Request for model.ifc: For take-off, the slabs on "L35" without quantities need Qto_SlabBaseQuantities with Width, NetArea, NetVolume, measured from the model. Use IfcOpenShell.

First a look at what the model holds.

```python
import ifcopenshell
import ifcopenshell.util.element
import ifcopenshell.util.unit

model = ifcopenshell.open("model.ifc")
print(model.schema)
for unit_type in ("LENGTHUNIT", "AREAUNIT", "VOLUMEUNIT"):
    print(unit_type, ifcopenshell.util.unit.calculate_unit_scale(model, unit_type))
storey = next(s for s in model.by_type("IfcBuildingStorey") if s.Name == "L35")
slabs = [e for e in ifcopenshell.util.element.get_decomposition(storey) if e.is_a("IfcSlab")]
for e in sorted(slabs, key=lambda e: e.id()):
    print(e.id(), e.is_a(), e.Name, list(ifcopenshell.util.element.get_psets(e, qtos_only=True)), sep=" | ")
```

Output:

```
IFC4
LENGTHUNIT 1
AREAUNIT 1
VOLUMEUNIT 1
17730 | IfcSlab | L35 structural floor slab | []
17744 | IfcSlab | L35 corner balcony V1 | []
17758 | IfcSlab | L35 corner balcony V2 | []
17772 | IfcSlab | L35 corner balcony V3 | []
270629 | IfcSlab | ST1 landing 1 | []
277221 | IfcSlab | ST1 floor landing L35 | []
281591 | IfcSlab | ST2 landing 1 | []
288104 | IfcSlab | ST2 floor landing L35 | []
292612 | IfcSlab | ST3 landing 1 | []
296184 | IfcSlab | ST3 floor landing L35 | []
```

```python
import ifcopenshell
import ifcopenshell.api.pset
import ifcopenshell.geom
import ifcopenshell.util.element
import ifcopenshell.util.shape
import ifcopenshell.util.unit

model = ifcopenshell.open("model.ifc")
unit_scale = ifcopenshell.util.unit.calculate_unit_scale(model)
area_scale = ifcopenshell.util.unit.calculate_unit_scale(model, "AREAUNIT")
volume_scale = ifcopenshell.util.unit.calculate_unit_scale(model, "VOLUMEUNIT")
settings = ifcopenshell.geom.settings()

storey = next(s for s in model.by_type("IfcBuildingStorey") if s.Name == "L35")
slabs = [e for e in ifcopenshell.util.element.get_decomposition(storey) if e.is_a("IfcSlab")]

for e in sorted(slabs, key=lambda e: e.id()):
    if ifcopenshell.util.element.get_psets(e, qtos_only=True, should_inherit=False):
        continue
    # Geometry comes back in metres, in the element's own axes.
    shape = ifcopenshell.geom.create_shape(settings, e)
    values = {
        "Width": ifcopenshell.util.shape.get_z(shape.geometry) / unit_scale,
        "NetArea": ifcopenshell.util.shape.get_footprint_area(shape.geometry) / area_scale,
        "NetVolume": ifcopenshell.util.shape.get_volume(shape.geometry) / volume_scale,
    }
    qto = ifcopenshell.api.pset.add_qto(model, product=e, name="Qto_SlabBaseQuantities")
    ifcopenshell.api.pset.edit_qto(model, qto=qto, properties=values)
    print(e.id(), {k: round(v, 3) for k, v in values.items()})

model.write("model-out.ifc")
```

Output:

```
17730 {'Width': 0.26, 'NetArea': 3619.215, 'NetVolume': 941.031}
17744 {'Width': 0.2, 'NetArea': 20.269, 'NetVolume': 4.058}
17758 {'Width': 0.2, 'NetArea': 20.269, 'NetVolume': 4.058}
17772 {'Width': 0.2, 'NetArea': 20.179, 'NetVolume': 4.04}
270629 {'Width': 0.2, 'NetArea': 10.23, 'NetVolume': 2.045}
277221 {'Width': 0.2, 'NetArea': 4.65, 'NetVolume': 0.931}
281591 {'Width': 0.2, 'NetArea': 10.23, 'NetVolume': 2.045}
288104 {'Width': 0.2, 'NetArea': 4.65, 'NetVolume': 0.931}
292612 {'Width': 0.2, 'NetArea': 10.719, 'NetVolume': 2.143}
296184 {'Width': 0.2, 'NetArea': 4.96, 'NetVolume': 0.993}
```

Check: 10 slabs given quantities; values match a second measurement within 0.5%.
